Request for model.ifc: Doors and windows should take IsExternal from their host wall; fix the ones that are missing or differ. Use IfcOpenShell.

First a look at what the model holds.

```python
import ifcopenshell
import ifcopenshell.util.element

model = ifcopenshell.open("model.ifc")
print(model.schema)
seen = {}
for e in model.by_type("IfcDoor") + model.by_type("IfcWindow"):
    if not e.FillsVoids:
        continue
    host = e.FillsVoids[0].RelatingOpeningElement.VoidsElements[0].RelatingBuildingElement
    own = ifcopenshell.util.element.get_pset(e, f"Pset_{e.is_a()[3:].removesuffix('StandardCase')}Common", "IsExternal")
    wall = ifcopenshell.util.element.get_pset(host, "Pset_WallCommon", "IsExternal")
    seen[e.is_a(), own, wall] = seen.get((e.is_a(), own, wall), 0) + 1
for (cls, own, wall), count in sorted(seen.items(), key=str):
    print(count, cls, "IsExternal:", own, "| host wall:", wall)
```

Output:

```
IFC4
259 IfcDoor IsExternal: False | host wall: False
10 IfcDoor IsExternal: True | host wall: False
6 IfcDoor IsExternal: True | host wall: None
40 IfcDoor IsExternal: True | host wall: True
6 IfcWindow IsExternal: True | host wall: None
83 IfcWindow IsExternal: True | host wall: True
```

```python
import ifcopenshell
import ifcopenshell.api.pset
import ifcopenshell.util.element

model = ifcopenshell.open("model.ifc")

count = 0
for ifc_class, pset_name in (("IfcDoor", "Pset_DoorCommon"), ("IfcWindow", "Pset_WindowCommon")):
    for e in model.by_type(ifc_class):
        if not e.FillsVoids:
            continue
        host = e.FillsVoids[0].RelatingOpeningElement.VoidsElements[0].RelatingBuildingElement
        external = ifcopenshell.util.element.get_pset(host, "Pset_WallCommon", "IsExternal")
        if external is None or ifcopenshell.util.element.get_pset(e, pset_name, "IsExternal") == external:
            continue
        pset = ifcopenshell.api.pset.add_pset(model, product=e, name=pset_name)
        ifcopenshell.api.pset.edit_pset(model, pset=pset, properties={"IsExternal": external})
        count += 1

print(count, "updated")

model.write("model_v2.ifc")
```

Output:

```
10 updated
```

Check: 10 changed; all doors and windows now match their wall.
